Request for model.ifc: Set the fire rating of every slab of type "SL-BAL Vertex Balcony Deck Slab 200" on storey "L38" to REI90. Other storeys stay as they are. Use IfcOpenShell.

First a look at what the model holds.

```python
import ifcopenshell
import ifcopenshell.util.element

model = ifcopenshell.open("model.ifc")
print(model.schema)
storey = next(s for s in model.by_type("IfcBuildingStorey") if s.Name == "L38")
slabs = [e for e in ifcopenshell.util.element.get_decomposition(storey) if e.is_a("IfcSlab")]
seen = {}
for e in slabs:
    element_type = ifcopenshell.util.element.get_type(e)
    key = (element_type.Name if element_type != e and element_type else None, ifcopenshell.util.element.get_pset(e, "Pset_SlabCommon", "FireRating"))
    seen[key] = seen.get(key, 0) + 1
for (name, value), count in sorted(seen.items(), key=str):
    print(count, "x", name, "|", value)
```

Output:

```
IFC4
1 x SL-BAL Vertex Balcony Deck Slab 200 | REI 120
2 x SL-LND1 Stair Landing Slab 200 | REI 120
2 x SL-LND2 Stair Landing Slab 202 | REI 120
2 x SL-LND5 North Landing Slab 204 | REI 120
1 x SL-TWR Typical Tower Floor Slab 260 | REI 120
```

```python
import ifcopenshell
import ifcopenshell.api.pset
import ifcopenshell.util.element

model = ifcopenshell.open("model.ifc")

storey = next(s for s in model.by_type("IfcBuildingStorey") if s.Name == "L38")
slabs = [e for e in ifcopenshell.util.element.get_decomposition(storey) if e.is_a("IfcSlab")]

count = 0
for e in slabs:
    element_type = ifcopenshell.util.element.get_type(e)
    if element_type in (None, e) or element_type.Name != "SL-BAL Vertex Balcony Deck Slab 200":
        continue
    found = ifcopenshell.util.element.get_pset(e, "Pset_SlabCommon", should_inherit=False)
    if found:
        pset = model.by_id(found["id"])
        if len(ifcopenshell.util.element.get_elements_by_pset(pset)) > 1:
            pset = ifcopenshell.api.pset.unshare_pset(model, products=[e], pset=pset)[0]
    else:
        pset = ifcopenshell.api.pset.add_pset(model, product=e, name="Pset_SlabCommon")
    ifcopenshell.api.pset.edit_pset(model, pset=pset, properties={"FireRating": "REI90"})
    count += 1

print(count, "slabs updated")

model.write("model_updated.ifc")
```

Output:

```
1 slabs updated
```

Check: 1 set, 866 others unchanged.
